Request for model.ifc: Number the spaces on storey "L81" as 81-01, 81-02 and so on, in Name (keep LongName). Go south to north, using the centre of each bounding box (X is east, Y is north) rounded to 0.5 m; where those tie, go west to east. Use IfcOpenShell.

First a look at what the model holds.

```python
import ifcopenshell
import ifcopenshell.util.element
import ifcopenshell.util.placement

model = ifcopenshell.open("model.ifc")
print(model.schema)
storey = next(s for s in model.by_type("IfcBuildingStorey") if s.Name == "L81")
spaces = [e for e in ifcopenshell.util.element.get_decomposition(storey) if e.is_a("IfcSpace")]
for e in sorted(spaces, key=lambda e: e.id()):
    origin = ifcopenshell.util.placement.get_local_placement(e.ObjectPlacement)[:3, 3]
    print(e.id(), e.Name, e.LongName, origin.round(2) + 0.0, sep=" | ")
```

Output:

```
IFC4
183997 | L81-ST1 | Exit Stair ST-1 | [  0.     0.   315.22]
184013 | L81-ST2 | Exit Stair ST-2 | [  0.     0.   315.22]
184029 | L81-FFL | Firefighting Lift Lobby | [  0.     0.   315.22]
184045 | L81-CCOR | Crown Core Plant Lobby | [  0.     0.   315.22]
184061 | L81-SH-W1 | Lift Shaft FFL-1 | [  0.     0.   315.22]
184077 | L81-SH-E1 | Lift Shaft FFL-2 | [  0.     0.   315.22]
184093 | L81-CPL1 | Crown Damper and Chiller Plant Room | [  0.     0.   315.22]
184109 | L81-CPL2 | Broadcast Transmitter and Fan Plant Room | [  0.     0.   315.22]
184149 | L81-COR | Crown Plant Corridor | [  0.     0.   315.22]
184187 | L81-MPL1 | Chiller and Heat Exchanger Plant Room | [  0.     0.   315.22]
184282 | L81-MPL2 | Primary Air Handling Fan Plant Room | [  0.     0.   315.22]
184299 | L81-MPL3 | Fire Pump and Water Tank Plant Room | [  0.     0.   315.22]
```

```python
import ifcopenshell
import ifcopenshell.geom
import ifcopenshell.util.element
import ifcopenshell.util.shape

model = ifcopenshell.open("model.ifc")
settings = ifcopenshell.geom.settings()
settings.set("use-world-coords", True)


def centre(element):
    shape = ifcopenshell.geom.create_shape(settings, element)
    return ifcopenshell.util.shape.get_bbox_centroid(shape.geometry)


storey = next(s for s in model.by_type("IfcBuildingStorey") if s.Name == "L81")
spaces = [e for e in ifcopenshell.util.element.get_decomposition(storey) if e.is_a("IfcSpace")]

# Insertion points can sit at a corner or the storey origin, so sort by the geometry (in metres).
centres = {e: centre(e) for e in spaces}
spaces.sort(key=lambda e: (round(centres[e][1] / 0.5), centres[e][0]))

for i, e in enumerate(spaces, start=1):
    number = f"81-{i:02d}"
    e.Name = number
    print(e.id(), number)

model.write("model_rev.ifc")
```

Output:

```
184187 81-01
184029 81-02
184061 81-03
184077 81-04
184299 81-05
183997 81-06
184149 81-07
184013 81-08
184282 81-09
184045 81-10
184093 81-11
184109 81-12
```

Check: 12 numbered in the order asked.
